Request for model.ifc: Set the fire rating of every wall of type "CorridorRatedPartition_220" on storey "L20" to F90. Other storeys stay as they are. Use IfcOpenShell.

First a look at what the model holds.

```python
import ifcopenshell
import ifcopenshell.util.element

model = ifcopenshell.open("model.ifc")
print(model.schema)
storey = next(s for s in model.by_type("IfcBuildingStorey") if s.Name == "L20")
walls = [e for e in ifcopenshell.util.element.get_decomposition(storey) if e.is_a("IfcWall")]
seen = {}
for e in walls:
    element_type = ifcopenshell.util.element.get_type(e)
    key = (element_type.Name if element_type != e and element_type else None, ifcopenshell.util.element.get_pset(e, "Pset_WallCommon", "FireRating"))
    seen[key] = seen.get(key, 0) + 1
for (name, value), count in sorted(seen.items(), key=str):
    print(count, "x", name, "|", value)
```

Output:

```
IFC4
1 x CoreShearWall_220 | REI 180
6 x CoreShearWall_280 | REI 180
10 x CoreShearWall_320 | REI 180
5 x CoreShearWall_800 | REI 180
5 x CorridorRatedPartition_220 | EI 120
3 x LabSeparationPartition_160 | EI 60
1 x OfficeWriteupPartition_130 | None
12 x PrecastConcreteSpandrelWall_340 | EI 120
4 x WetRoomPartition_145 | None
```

```python
import ifcopenshell
import ifcopenshell.api.pset
import ifcopenshell.util.element

model = ifcopenshell.open("model.ifc")

storey = next(s for s in model.by_type("IfcBuildingStorey") if s.Name == "L20")
walls = [e for e in ifcopenshell.util.element.get_decomposition(storey) if e.is_a("IfcWall")]

count = 0
for e in walls:
    element_type = ifcopenshell.util.element.get_type(e)
    if element_type in (None, e) or element_type.Name != "CorridorRatedPartition_220":
        continue
    # add_pset returns the element's existing set when there is one.
    pset = ifcopenshell.api.pset.add_pset(model, product=e, name="Pset_WallCommon")
    ifcopenshell.api.pset.edit_pset(model, pset=pset, properties={"FireRating": "F90"})
    count += 1

print(count, "walls updated")

model.write("model_rev.ifc")
```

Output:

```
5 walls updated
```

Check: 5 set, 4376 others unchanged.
